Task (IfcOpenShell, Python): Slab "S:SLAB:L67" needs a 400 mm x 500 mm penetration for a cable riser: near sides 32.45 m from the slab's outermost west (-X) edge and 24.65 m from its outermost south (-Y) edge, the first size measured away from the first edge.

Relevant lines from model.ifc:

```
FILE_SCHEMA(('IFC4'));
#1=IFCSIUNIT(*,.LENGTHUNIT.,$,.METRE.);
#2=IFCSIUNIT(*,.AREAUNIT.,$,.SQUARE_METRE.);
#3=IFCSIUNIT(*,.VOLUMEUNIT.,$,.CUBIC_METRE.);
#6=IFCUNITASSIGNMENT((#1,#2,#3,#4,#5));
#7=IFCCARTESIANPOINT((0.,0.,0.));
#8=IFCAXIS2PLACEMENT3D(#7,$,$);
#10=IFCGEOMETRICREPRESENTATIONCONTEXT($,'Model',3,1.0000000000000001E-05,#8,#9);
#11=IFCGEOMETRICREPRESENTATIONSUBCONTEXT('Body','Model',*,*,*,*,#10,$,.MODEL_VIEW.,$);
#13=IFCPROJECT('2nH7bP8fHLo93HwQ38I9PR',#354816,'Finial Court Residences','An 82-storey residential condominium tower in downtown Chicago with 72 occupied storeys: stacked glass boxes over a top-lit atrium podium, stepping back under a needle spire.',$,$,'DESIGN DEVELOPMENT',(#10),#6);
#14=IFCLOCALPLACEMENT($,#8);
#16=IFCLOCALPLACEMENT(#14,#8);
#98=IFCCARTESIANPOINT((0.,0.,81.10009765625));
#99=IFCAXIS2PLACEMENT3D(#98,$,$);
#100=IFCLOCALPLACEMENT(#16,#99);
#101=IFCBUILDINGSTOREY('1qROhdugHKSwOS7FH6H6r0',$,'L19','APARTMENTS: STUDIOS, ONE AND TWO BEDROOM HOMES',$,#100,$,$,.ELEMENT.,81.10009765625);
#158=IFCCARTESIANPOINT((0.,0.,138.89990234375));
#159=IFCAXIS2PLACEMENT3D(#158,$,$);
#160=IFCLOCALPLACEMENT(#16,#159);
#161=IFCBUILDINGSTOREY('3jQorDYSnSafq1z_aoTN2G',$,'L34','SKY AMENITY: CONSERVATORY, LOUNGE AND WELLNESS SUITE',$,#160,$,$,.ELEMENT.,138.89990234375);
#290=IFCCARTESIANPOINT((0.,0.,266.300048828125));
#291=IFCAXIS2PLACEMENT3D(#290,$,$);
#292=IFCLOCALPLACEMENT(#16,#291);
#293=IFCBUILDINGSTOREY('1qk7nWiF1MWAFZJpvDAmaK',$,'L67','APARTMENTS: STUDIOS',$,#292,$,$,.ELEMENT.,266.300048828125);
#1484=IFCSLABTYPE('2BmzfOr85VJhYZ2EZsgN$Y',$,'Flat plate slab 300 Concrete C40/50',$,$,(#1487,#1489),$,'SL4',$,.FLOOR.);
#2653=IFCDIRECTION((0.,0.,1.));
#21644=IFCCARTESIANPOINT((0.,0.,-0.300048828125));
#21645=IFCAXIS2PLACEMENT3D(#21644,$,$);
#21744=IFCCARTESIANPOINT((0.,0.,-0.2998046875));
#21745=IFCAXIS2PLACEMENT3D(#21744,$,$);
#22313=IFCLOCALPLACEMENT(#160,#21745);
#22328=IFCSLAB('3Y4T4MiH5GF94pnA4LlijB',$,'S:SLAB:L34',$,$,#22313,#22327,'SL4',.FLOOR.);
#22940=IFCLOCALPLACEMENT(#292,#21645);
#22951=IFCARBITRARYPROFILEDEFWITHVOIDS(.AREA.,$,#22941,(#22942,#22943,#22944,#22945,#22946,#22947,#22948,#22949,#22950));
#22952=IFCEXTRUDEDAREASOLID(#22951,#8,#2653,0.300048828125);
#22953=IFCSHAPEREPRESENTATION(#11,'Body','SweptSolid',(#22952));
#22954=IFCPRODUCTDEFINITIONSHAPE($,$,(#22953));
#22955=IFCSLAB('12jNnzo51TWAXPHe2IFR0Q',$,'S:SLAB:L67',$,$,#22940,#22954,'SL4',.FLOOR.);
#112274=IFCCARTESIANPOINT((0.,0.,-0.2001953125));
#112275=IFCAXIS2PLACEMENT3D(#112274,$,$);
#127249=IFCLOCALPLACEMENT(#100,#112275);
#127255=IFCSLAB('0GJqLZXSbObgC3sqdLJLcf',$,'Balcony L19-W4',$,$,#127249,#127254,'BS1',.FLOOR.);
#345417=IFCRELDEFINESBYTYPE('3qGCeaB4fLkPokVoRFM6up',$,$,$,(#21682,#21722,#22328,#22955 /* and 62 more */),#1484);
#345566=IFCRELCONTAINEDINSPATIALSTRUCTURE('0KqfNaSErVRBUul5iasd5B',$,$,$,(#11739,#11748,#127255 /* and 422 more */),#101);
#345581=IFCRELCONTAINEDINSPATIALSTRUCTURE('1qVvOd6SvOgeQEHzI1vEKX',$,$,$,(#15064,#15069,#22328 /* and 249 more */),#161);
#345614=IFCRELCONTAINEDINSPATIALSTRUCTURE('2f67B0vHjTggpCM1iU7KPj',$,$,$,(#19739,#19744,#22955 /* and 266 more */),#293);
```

```python
import numpy as np
import ifcopenshell
import ifcopenshell.api.feature
import ifcopenshell.api.geometry
import ifcopenshell.api.root
import ifcopenshell.geom
import ifcopenshell.util.placement
import ifcopenshell.util.representation
import ifcopenshell.util.shape
import ifcopenshell.util.unit

model = ifcopenshell.open("model.ifc")
unit_scale = ifcopenshell.util.unit.calculate_unit_scale(model)
settings = ifcopenshell.geom.settings()


def volume(element):
    """Net volume in cubic metres, openings subtracted."""
    shape = ifcopenshell.geom.create_shape(settings, element)
    return ifcopenshell.util.shape.get_volume(shape.geometry)


slab = model.by_guid("12jNnzo51TWAXPHe2IFR0Q")
before = volume(slab)

# Extent in the slab's own axes, in metres. The edges named are its -X and -Y sides.
slab_shape = ifcopenshell.geom.create_shape(settings, slab)
vertices = ifcopenshell.util.shape.get_vertices(slab_shape.geometry)
x_min, y_min, bottom = vertices.min(axis=0)
top = vertices[:, 2].max()

opening = ifcopenshell.api.root.create_entity(model, ifc_class="IfcOpeningElement", name="Cable riser opening", predefined_type="OPENING")
context = ifcopenshell.util.representation.get_context(model, "Model", "Body", "MODEL_VIEW")
width, depth = 0.4, 0.5
outline = [(0.0, 0.0), (width, 0.0), (width, depth), (0.0, depth), (0.0, 0.0)]
# Overshoot both faces by 50 mm so the cut is clean.
shape = ifcopenshell.api.geometry.add_slab_representation(
    model, context=context, depth=top - bottom + 0.1, polyline=outline
)
ifcopenshell.api.geometry.assign_representation(model, product=opening, representation=shape)

matrix = ifcopenshell.util.placement.get_local_placement(slab.ObjectPlacement)
matrix[:, 3] = matrix @ np.append(np.array([x_min + 32.45, y_min + 24.65, bottom - 0.05]) / unit_scale, 1.0)
ifcopenshell.api.geometry.edit_object_placement(model, product=opening, matrix=matrix, is_si=False)
ifcopenshell.api.feature.add_feature(model, feature=opening, element=slab)

after = volume(slab)

print(f"slab volume {before:.3f} -> {after:.3f} m3")

model.write("model_updated.ifc")
```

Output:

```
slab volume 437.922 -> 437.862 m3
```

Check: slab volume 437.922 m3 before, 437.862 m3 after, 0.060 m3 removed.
